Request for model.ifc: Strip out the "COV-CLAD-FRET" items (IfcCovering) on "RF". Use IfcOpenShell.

First a look at what the model holds.

```python
import ifcopenshell
import ifcopenshell.util.element

model = ifcopenshell.open("model.ifc")
print(model.schema)
storey = next(s for s in model.by_type("IfcBuildingStorey") if s.Name == "RF")
coverings = [e for e in ifcopenshell.util.element.get_decomposition(storey) if e.is_a("IfcCovering")]
seen = {}
for e in coverings:
    element_type = ifcopenshell.util.element.get_type(e)
    name = element_type.Name if element_type not in (None, e) else None
    seen[name] = seen.get(name, 0) + 1
for name, count in sorted(seen.items(), key=str):
    print(count, "x", name)
```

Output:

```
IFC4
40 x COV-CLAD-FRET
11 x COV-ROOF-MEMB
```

```python
import ifcopenshell
import ifcopenshell.api.root
import ifcopenshell.util.element

model = ifcopenshell.open("model.ifc")

storey = next(s for s in model.by_type("IfcBuildingStorey") if s.Name == "RF")
coverings = [e for e in ifcopenshell.util.element.get_decomposition(storey) if e.is_a("IfcCovering")]
targets = [e for e in coverings if (t := ifcopenshell.util.element.get_type(e)) not in (None, e) and t.Name == "COV-CLAD-FRET"]

for e in targets:
    ifcopenshell.api.root.remove_product(model, product=e)
print(len(targets), "removed")

model.write("model_v2.ifc")
```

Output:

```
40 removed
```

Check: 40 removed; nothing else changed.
